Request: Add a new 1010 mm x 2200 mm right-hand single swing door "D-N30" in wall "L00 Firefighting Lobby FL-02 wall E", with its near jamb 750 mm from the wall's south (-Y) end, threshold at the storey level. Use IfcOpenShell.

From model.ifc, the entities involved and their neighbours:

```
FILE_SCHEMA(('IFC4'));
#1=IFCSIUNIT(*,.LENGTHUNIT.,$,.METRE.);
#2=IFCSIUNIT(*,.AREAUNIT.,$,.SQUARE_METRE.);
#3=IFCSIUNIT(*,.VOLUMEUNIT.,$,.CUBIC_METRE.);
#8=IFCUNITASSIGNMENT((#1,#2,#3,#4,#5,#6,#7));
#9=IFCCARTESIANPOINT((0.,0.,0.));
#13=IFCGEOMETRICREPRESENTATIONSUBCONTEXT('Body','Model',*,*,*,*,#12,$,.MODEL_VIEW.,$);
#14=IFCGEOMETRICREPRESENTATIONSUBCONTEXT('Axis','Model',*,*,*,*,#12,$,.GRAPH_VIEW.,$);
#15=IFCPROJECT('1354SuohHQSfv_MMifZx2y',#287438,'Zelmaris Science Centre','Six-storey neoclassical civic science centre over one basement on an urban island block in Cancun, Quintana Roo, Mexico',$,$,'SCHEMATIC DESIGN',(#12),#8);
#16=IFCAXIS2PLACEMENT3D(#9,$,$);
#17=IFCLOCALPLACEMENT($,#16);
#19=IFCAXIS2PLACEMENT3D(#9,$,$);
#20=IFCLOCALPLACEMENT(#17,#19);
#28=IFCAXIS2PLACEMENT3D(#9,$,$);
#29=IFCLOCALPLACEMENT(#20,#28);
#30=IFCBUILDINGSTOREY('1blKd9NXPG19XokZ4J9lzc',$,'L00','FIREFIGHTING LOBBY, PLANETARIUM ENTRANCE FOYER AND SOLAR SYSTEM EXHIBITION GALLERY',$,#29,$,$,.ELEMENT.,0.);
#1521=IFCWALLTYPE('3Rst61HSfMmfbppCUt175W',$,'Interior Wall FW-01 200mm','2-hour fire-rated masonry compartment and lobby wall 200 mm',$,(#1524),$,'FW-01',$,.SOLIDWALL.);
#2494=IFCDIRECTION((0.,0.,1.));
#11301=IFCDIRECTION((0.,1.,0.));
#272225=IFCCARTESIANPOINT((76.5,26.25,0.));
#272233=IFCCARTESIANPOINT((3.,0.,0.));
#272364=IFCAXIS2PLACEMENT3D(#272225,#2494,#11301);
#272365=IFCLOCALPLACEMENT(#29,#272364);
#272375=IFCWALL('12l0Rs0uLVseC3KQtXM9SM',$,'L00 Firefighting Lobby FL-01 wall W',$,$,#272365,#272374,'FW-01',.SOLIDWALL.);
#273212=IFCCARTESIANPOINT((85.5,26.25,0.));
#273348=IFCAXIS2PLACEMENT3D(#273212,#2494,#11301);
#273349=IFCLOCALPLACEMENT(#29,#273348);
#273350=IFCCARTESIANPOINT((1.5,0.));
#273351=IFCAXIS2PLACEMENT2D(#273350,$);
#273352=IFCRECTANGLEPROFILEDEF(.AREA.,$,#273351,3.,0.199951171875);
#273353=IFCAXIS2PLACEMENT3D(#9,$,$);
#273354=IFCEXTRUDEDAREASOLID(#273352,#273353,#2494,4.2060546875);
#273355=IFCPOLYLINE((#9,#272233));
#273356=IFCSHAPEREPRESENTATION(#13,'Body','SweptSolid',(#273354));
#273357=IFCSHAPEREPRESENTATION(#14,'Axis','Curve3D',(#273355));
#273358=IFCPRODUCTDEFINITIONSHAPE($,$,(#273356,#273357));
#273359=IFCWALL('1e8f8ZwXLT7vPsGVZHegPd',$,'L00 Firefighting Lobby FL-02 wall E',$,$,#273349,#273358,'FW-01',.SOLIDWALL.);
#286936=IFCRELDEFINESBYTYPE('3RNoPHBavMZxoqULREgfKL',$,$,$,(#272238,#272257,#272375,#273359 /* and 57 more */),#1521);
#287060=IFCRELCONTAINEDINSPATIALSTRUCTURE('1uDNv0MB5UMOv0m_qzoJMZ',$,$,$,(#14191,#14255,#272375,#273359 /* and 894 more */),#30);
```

```python
import numpy as np
import ifcopenshell
import ifcopenshell.api.feature
import ifcopenshell.api.geometry
import ifcopenshell.api.root
import ifcopenshell.api.spatial
import ifcopenshell.geom
import ifcopenshell.util.element
import ifcopenshell.util.placement
import ifcopenshell.util.representation
import ifcopenshell.util.shape
import ifcopenshell.util.unit

model = ifcopenshell.open("model.ifc")
unit_scale = ifcopenshell.util.unit.calculate_unit_scale(model)
settings = ifcopenshell.geom.settings()


def volume(element):
    """Net volume in cubic metres, openings subtracted."""
    shape = ifcopenshell.geom.create_shape(settings, element)
    return ifcopenshell.util.shape.get_volume(shape.geometry)


wall = model.by_guid("1e8f8ZwXLT7vPsGVZHegPd")
storey = ifcopenshell.util.element.get_container(wall, ifc_class="IfcBuildingStorey")
context = ifcopenshell.util.representation.get_context(model, "Model", "Body", "MODEL_VIEW")
before = volume(wall)

width, height, from_end, sill = 1.01, 2.2, 0.75, 0.0  # metres

# The wall runs along its own X axis, and the end named is its -X end.
wall_shape = ifcopenshell.geom.create_shape(settings, wall)
x, y, z = ifcopenshell.util.shape.get_vertices(wall_shape.geometry).T
start = x.min() + from_end
face, thickness = float(y.min()), float(y.max() - y.min())
wall_matrix = ifcopenshell.util.placement.get_local_placement(wall.ObjectPlacement)
level = ifcopenshell.util.placement.get_local_placement(storey.ObjectPlacement)[2, 3]


def in_wall(x, y):
    """Placement at x, y metres in the wall's axes, at sill height."""
    matrix = wall_matrix.copy()
    matrix[:, 3] = wall_matrix @ np.array([x / unit_scale, y / unit_scale, 0.0, 1.0])
    matrix[2, 3] = level + sill / unit_scale
    return matrix


# Opening: a box that overshoots both wall faces by 50 mm.
opening = ifcopenshell.api.root.create_entity(model, ifc_class="IfcOpeningElement", predefined_type="OPENING")
box = ifcopenshell.api.geometry.add_wall_representation(
    model, context=context, length=width, height=height, thickness=thickness + 0.1
)
ifcopenshell.api.geometry.assign_representation(model, product=opening, representation=box)
ifcopenshell.api.geometry.edit_object_placement(model, product=opening, matrix=in_wall(start, face - 0.05), is_si=False)
ifcopenshell.api.feature.add_feature(model, feature=opening, element=wall)

door = ifcopenshell.api.root.create_entity(model, ifc_class="IfcDoor", name="D-N30", predefined_type="DOOR")
door.OverallWidth, door.OverallHeight = width / unit_scale, height / unit_scale
door.OperationType = "SINGLE_SWING_RIGHT"
body = ifcopenshell.api.geometry.add_door_representation(
    model,
    context=context,
    overall_width=door.OverallWidth,
    overall_height=door.OverallHeight,
    operation_type="SINGLE_SWING_RIGHT",
    lining_properties={"LiningDepth": thickness / unit_scale, "ThresholdDepth": thickness / unit_scale},
)
ifcopenshell.api.geometry.assign_representation(model, product=door, representation=body)
ifcopenshell.api.spatial.assign_container(model, products=[door], relating_structure=storey)
ifcopenshell.api.feature.add_filling(model, opening=opening, element=door)

# The lining spans the wall, so the door starts at the wall face.
ifcopenshell.api.geometry.edit_object_placement(model, product=door, matrix=in_wall(start, face), is_si=False)

after = volume(wall)

print(f"wall volume {before:.3f} -> {after:.3f} m3")

model.write("model_edited.ifc")
```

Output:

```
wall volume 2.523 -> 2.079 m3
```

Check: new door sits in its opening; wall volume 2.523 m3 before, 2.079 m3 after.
